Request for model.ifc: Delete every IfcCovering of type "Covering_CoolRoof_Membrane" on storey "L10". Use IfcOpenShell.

First a look at what the model holds.

```python
import ifcopenshell
import ifcopenshell.util.element

model = ifcopenshell.open("model.ifc")
print(model.schema)
storey = next(s for s in model.by_type("IfcBuildingStorey") if s.Name == "L10")
coverings = [e for e in ifcopenshell.util.element.get_decomposition(storey) if e.is_a("IfcCovering")]
seen = {}
for e in coverings:
    element_type = ifcopenshell.util.element.get_type(e)
    name = element_type.Name if element_type not in (None, e) else None
    seen[name] = seen.get(name, 0) + 1
for name, count in sorted(seen.items(), key=str):
    print(count, "x", name)
```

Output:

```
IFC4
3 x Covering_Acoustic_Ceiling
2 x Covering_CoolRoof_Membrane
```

```python
import ifcopenshell
import ifcopenshell.api.root
import ifcopenshell.util.element

model = ifcopenshell.open("model.ifc")

storey = next(s for s in model.by_type("IfcBuildingStorey") if s.Name == "L10")
coverings = [e for e in ifcopenshell.util.element.get_decomposition(storey) if e.is_a("IfcCovering")]
targets = [e for e in coverings if (t := ifcopenshell.util.element.get_type(e)) not in (None, e) and t.Name == "Covering_CoolRoof_Membrane"]

for e in targets:
    ifcopenshell.api.root.remove_product(model, product=e)
print(len(targets), "removed")

model.write("model-out.ifc")
```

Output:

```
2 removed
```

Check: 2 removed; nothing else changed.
